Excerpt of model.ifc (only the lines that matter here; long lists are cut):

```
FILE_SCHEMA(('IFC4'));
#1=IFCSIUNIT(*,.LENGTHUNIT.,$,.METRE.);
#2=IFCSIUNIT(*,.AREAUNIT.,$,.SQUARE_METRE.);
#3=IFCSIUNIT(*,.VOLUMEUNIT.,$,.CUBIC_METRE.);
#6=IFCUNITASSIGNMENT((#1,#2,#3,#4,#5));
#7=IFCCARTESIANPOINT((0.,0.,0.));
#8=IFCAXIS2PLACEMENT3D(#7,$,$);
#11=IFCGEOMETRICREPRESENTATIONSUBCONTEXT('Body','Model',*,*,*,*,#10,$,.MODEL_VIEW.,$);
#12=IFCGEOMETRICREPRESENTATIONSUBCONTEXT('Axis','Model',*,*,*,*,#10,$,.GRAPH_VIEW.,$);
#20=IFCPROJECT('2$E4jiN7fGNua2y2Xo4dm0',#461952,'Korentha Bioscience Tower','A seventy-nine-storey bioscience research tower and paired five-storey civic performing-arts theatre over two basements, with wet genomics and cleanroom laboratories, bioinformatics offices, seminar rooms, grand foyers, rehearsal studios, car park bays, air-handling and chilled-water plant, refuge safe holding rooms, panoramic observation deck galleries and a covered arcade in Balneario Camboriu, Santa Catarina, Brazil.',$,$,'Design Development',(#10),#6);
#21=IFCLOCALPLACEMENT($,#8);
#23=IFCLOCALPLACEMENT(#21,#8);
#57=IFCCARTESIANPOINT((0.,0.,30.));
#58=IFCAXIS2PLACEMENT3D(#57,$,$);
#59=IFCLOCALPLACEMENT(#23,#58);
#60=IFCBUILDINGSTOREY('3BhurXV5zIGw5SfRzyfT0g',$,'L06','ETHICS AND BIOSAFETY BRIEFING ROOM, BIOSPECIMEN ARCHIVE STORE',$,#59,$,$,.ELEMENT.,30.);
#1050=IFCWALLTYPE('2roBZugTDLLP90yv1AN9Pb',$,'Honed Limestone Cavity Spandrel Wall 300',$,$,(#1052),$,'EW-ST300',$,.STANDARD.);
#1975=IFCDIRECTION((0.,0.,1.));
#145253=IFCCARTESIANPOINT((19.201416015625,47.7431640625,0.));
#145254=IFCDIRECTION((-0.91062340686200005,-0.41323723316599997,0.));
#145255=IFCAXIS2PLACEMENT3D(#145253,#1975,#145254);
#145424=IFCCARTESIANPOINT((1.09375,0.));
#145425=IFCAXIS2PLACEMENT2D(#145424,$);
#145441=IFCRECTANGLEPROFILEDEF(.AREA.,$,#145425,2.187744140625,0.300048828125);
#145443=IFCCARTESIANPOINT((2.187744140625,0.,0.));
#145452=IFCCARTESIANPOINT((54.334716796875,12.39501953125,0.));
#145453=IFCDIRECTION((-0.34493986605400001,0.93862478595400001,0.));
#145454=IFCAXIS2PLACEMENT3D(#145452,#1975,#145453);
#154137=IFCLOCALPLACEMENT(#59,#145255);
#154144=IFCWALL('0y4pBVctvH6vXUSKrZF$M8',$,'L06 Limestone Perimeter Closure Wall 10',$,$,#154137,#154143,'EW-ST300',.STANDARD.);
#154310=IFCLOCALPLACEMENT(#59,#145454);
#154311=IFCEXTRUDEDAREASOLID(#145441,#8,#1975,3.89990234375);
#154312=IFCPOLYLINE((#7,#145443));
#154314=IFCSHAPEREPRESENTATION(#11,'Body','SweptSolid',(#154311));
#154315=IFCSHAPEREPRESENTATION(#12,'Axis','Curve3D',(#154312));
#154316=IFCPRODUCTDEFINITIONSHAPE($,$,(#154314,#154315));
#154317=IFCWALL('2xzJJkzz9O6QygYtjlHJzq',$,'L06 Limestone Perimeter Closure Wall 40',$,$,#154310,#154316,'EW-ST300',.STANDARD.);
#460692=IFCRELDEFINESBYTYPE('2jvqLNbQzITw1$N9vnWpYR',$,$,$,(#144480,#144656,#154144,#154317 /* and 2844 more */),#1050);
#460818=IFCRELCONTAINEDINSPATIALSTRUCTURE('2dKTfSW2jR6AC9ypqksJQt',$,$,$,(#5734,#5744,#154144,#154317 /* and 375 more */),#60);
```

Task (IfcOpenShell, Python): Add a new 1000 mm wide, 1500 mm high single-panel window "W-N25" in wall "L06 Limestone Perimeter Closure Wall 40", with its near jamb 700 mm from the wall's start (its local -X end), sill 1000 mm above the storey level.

```python
import numpy as np
import ifcopenshell
import ifcopenshell.api.feature
import ifcopenshell.api.geometry
import ifcopenshell.api.root
import ifcopenshell.api.spatial
import ifcopenshell.geom
import ifcopenshell.util.element
import ifcopenshell.util.placement
import ifcopenshell.util.representation
import ifcopenshell.util.shape
import ifcopenshell.util.unit

model = ifcopenshell.open("model.ifc")
unit_scale = ifcopenshell.util.unit.calculate_unit_scale(model)
settings = ifcopenshell.geom.settings()


def volume(element):
    """Net volume in cubic metres, openings subtracted."""
    shape = ifcopenshell.geom.create_shape(settings, element)
    return ifcopenshell.util.shape.get_volume(shape.geometry)


wall = model.by_guid("2xzJJkzz9O6QygYtjlHJzq")
storey = ifcopenshell.util.element.get_container(wall, ifc_class="IfcBuildingStorey")
context = ifcopenshell.util.representation.get_context(model, "Model", "Body", "MODEL_VIEW")
before = volume(wall)

width, height, from_end, sill = 1, 1.5, 0.7, 1  # metres

# The wall runs along its own X axis, and the end named is its -X end.
wall_shape = ifcopenshell.geom.create_shape(settings, wall)
x, y, z = ifcopenshell.util.shape.get_vertices(wall_shape.geometry).T
start = x.min() + from_end
face, thickness = float(y.min()), float(y.max() - y.min())
wall_matrix = ifcopenshell.util.placement.get_local_placement(wall.ObjectPlacement)
level = ifcopenshell.util.placement.get_local_placement(storey.ObjectPlacement)[2, 3]


def in_wall(x, y):
    """Placement at x, y metres in the wall's axes, at sill height."""
    matrix = wall_matrix.copy()
    matrix[:, 3] = wall_matrix @ np.array([x / unit_scale, y / unit_scale, 0.0, 1.0])
    matrix[2, 3] = level + sill / unit_scale
    return matrix


# Opening: a box that overshoots both wall faces by 50 mm.
opening = ifcopenshell.api.root.create_entity(model, ifc_class="IfcOpeningElement", predefined_type="OPENING")
box = ifcopenshell.api.geometry.add_wall_representation(
    model, context=context, length=width, height=height, thickness=thickness + 0.1
)
ifcopenshell.api.geometry.assign_representation(model, product=opening, representation=box)
ifcopenshell.api.geometry.edit_object_placement(model, product=opening, matrix=in_wall(start, face - 0.05), is_si=False)
ifcopenshell.api.feature.add_feature(model, feature=opening, element=wall)

window = ifcopenshell.api.root.create_entity(model, ifc_class="IfcWindow", name="W-N25", predefined_type="WINDOW")
window.OverallWidth, window.OverallHeight = width / unit_scale, height / unit_scale
window.PartitioningType = "SINGLE_PANEL"
body = ifcopenshell.api.geometry.add_window_representation(
    model,
    context=context,
    overall_width=window.OverallWidth,
    overall_height=window.OverallHeight,
    partition_type="SINGLE_PANEL",
)
ifcopenshell.api.geometry.assign_representation(model, product=window, representation=body)
ifcopenshell.api.spatial.assign_container(model, products=[window], relating_structure=storey)
ifcopenshell.api.feature.add_filling(model, opening=opening, element=window)

# Centre the window in the wall's thickness.
ifcopenshell.api.geometry.edit_object_placement(model, product=window, matrix=in_wall(start, face), is_si=False)
window_shape = ifcopenshell.geom.create_shape(settings, window)
depth = ifcopenshell.util.shape.get_vertices(window_shape.geometry)[:, 1]
offset = face + thickness / 2 - (depth.min() + depth.max()) / 2
ifcopenshell.api.geometry.edit_object_placement(model, product=window, matrix=in_wall(start, offset), is_si=False)

after = volume(wall)

print(f"wall volume {before:.3f} -> {after:.3f} m3")

model.write("model_rev.ifc")
```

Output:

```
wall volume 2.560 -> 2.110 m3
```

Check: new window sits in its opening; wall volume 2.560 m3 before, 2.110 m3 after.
